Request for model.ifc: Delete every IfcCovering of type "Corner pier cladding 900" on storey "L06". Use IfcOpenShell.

First a look at what the model holds.

```python
import ifcopenshell
import ifcopenshell.util.element

model = ifcopenshell.open("model.ifc")
print(model.schema)
storey = next(s for s in model.by_type("IfcBuildingStorey") if s.Name == "L06")
coverings = [e for e in ifcopenshell.util.element.get_decomposition(storey) if e.is_a("IfcCovering")]
seen = {}
for e in coverings:
    element_type = ifcopenshell.util.element.get_type(e)
    name = element_type.Name if element_type not in (None, e) else None
    seen[name] = seen.get(name, 0) + 1
for name, count in sorted(seen.items(), key=str):
    print(count, "x", name)
```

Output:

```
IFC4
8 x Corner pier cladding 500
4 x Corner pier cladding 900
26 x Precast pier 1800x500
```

```python
import ifcopenshell
import ifcopenshell.api.root
import ifcopenshell.util.element

model = ifcopenshell.open("model.ifc")

storey = next(s for s in model.by_type("IfcBuildingStorey") if s.Name == "L06")
coverings = [e for e in ifcopenshell.util.element.get_decomposition(storey) if e.is_a("IfcCovering")]
targets = [e for e in coverings if (t := ifcopenshell.util.element.get_type(e)) not in (None, e) and t.Name == "Corner pier cladding 900"]

for e in targets:
    ifcopenshell.api.root.remove_product(model, product=e)
print(len(targets), "removed")

model.write("model_updated.ifc")
```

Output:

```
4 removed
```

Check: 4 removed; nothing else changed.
